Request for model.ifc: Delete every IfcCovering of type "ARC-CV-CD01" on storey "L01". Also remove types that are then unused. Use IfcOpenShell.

First a look at what the model holds.

```python
import ifcopenshell
import ifcopenshell.util.element

model = ifcopenshell.open("model.ifc")
print(model.schema)
storey = next(s for s in model.by_type("IfcBuildingStorey") if s.Name == "L01")
coverings = [e for e in ifcopenshell.util.element.get_decomposition(storey) if e.is_a("IfcCovering")]
seen = {}
for e in coverings:
    element_type = ifcopenshell.util.element.get_type(e)
    name = element_type.Name if element_type not in (None, e) else None
    seen[name] = seen.get(name, 0) + 1
for name, count in sorted(seen.items(), key=str):
    print(count, "x", name)
```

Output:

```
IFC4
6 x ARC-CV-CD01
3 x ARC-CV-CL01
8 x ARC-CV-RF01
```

```python
import ifcopenshell
import ifcopenshell.api.root
import ifcopenshell.util.element

model = ifcopenshell.open("model.ifc")

storey = next(s for s in model.by_type("IfcBuildingStorey") if s.Name == "L01")
coverings = [e for e in ifcopenshell.util.element.get_decomposition(storey) if e.is_a("IfcCovering")]
targets = [e for e in coverings if (t := ifcopenshell.util.element.get_type(e)) not in (None, e) and t.Name == "ARC-CV-CD01"]
types = {ifcopenshell.util.element.get_type(e) for e in targets} - {None, *targets}

for e in targets:
    ifcopenshell.api.root.remove_product(model, product=e)
print(len(targets), "removed")

unused = [t for t in types if not ifcopenshell.util.element.get_types(t)]
for t in unused:
    ifcopenshell.api.root.remove_product(model, product=t)
print(len(unused), "unused types removed")

model.write("model-out.ifc")
```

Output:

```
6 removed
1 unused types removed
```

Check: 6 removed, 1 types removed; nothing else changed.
